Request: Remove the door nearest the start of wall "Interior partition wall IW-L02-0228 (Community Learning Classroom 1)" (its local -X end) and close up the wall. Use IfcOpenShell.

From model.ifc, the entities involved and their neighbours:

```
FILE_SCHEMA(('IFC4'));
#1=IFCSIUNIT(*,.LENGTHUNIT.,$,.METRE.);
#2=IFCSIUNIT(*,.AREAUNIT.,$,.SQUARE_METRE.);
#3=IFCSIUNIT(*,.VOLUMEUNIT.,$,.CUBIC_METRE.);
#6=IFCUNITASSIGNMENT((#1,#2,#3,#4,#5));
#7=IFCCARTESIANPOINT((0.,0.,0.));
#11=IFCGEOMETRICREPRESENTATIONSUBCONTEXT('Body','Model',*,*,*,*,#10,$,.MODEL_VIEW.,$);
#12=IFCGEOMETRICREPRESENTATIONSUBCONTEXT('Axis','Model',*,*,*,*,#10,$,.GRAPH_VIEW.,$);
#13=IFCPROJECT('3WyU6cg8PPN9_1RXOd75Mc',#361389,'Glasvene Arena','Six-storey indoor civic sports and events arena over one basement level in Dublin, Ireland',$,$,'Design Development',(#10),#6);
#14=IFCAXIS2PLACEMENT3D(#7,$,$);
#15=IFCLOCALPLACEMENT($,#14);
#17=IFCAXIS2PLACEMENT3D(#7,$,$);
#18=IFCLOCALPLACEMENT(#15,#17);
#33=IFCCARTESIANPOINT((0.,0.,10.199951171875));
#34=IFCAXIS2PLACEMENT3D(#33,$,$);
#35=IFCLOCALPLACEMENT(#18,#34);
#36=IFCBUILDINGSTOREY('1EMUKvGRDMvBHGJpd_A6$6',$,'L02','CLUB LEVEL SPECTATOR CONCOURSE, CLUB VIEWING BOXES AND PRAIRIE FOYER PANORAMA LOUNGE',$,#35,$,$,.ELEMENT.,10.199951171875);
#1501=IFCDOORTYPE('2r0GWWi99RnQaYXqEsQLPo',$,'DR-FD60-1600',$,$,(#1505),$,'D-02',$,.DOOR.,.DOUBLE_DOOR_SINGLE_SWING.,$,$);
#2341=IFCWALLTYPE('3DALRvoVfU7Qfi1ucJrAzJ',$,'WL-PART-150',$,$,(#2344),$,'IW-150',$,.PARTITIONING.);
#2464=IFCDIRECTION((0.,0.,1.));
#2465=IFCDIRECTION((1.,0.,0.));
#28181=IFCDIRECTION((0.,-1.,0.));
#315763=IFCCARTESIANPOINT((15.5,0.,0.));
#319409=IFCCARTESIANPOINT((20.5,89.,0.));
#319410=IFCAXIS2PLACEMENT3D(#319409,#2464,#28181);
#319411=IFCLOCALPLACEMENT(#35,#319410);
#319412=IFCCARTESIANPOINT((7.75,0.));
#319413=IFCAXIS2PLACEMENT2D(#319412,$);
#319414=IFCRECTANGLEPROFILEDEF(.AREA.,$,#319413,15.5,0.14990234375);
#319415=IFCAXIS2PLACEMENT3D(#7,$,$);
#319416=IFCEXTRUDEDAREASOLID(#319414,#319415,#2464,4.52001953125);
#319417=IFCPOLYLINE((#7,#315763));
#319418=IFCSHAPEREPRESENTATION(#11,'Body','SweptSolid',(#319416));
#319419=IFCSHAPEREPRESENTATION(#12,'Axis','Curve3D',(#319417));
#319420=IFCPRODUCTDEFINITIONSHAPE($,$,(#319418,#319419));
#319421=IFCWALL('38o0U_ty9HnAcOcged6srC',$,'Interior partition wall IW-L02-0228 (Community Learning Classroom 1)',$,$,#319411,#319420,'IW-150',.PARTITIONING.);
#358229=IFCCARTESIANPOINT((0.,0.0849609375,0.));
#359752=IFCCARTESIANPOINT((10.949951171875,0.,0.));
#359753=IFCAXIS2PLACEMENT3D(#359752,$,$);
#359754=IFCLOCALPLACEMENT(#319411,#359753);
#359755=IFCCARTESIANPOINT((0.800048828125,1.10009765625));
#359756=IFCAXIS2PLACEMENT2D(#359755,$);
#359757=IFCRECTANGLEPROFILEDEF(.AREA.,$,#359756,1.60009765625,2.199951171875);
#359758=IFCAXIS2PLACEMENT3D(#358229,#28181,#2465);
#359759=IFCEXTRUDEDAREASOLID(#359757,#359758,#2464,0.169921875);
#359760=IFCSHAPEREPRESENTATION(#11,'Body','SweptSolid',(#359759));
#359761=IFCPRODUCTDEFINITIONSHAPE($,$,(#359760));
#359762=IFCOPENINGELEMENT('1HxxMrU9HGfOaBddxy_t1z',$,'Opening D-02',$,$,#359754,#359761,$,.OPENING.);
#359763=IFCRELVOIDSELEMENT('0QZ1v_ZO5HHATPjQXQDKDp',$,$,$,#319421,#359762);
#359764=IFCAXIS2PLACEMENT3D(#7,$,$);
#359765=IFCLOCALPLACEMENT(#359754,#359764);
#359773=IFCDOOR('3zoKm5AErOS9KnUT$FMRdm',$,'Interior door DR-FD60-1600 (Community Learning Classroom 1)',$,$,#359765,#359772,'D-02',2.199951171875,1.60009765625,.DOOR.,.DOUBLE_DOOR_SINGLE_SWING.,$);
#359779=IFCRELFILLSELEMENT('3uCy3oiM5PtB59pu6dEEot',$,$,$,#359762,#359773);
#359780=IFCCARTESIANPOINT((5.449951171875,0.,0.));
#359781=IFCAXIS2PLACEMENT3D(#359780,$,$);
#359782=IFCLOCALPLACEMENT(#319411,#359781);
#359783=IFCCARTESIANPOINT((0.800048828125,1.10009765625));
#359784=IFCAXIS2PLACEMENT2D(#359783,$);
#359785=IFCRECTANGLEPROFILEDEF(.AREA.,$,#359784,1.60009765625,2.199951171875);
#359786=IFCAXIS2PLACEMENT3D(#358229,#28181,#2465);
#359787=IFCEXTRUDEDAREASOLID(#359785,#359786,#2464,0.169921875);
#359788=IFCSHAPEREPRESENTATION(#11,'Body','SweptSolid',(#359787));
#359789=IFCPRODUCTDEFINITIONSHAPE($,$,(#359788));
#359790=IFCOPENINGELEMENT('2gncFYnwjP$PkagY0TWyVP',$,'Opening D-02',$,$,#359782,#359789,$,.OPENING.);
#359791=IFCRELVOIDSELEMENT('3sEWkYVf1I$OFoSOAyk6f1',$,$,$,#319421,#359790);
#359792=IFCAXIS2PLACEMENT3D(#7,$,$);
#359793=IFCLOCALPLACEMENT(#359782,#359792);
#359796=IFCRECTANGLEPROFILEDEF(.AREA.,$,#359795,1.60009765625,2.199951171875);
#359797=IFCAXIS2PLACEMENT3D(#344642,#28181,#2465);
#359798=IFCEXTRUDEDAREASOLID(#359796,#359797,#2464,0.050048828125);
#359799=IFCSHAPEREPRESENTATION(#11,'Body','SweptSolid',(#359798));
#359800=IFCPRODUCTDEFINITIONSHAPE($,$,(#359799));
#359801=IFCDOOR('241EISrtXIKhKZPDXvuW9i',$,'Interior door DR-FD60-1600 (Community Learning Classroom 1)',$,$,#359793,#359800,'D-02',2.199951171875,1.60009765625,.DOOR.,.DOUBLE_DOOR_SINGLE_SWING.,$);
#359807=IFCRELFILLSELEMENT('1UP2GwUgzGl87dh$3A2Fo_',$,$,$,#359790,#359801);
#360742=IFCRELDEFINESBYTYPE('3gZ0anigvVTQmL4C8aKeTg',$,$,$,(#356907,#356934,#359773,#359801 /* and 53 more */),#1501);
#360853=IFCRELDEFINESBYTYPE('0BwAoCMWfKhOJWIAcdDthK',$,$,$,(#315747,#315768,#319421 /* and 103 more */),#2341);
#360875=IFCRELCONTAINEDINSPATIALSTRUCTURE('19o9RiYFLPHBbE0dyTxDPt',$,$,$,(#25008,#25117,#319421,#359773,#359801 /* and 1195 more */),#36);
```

```python
import ifcopenshell
import ifcopenshell.api.feature
import ifcopenshell.api.root
import ifcopenshell.geom
import ifcopenshell.util.shape

model = ifcopenshell.open("model.ifc")
settings = ifcopenshell.geom.settings()


def volume(element):
    """Net volume in cubic metres, openings subtracted."""
    shape = ifcopenshell.geom.create_shape(settings, element)
    return ifcopenshell.util.shape.get_volume(shape.geometry)


door = model.by_guid("241EISrtXIKhKZPDXvuW9i")
opening = door.FillsVoids[0].RelatingOpeningElement
wall = opening.VoidsElements[0].RelatingBuildingElement
before = volume(wall)

ifcopenshell.api.root.remove_product(model, product=door)
ifcopenshell.api.feature.remove_feature(model, feature=opening)

after = volume(wall)

print(f"wall volume {before:.3f} -> {after:.3f} m3")

model.write("model_edited.ifc")
```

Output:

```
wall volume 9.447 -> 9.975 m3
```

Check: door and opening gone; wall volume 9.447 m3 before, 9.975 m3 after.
